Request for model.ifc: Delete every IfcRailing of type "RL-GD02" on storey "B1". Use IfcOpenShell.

First a look at what the model holds.

```python
import ifcopenshell
import ifcopenshell.util.element

model = ifcopenshell.open("model.ifc")
print(model.schema)
storey = next(s for s in model.by_type("IfcBuildingStorey") if s.Name == "B1")
railings = [e for e in ifcopenshell.util.element.get_decomposition(storey) if e.is_a("IfcRailing")]
seen = {}
for e in railings:
    element_type = ifcopenshell.util.element.get_type(e)
    name = element_type.Name if element_type not in (None, e) else None
    seen[name] = seen.get(name, 0) + 1
for name, count in sorted(seen.items(), key=str):
    print(count, "x", name)
```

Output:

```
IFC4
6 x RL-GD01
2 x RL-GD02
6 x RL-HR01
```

```python
import ifcopenshell
import ifcopenshell.api.root
import ifcopenshell.util.element

model = ifcopenshell.open("model.ifc")

storey = next(s for s in model.by_type("IfcBuildingStorey") if s.Name == "B1")
railings = [e for e in ifcopenshell.util.element.get_decomposition(storey) if e.is_a("IfcRailing")]
targets = [e for e in railings if (t := ifcopenshell.util.element.get_type(e)) not in (None, e) and t.Name == "RL-GD02"]

for e in targets:
    ifcopenshell.api.root.remove_product(model, product=e)
print(len(targets), "removed")

model.write("model_edited.ifc")
```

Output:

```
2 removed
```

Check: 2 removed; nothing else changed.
